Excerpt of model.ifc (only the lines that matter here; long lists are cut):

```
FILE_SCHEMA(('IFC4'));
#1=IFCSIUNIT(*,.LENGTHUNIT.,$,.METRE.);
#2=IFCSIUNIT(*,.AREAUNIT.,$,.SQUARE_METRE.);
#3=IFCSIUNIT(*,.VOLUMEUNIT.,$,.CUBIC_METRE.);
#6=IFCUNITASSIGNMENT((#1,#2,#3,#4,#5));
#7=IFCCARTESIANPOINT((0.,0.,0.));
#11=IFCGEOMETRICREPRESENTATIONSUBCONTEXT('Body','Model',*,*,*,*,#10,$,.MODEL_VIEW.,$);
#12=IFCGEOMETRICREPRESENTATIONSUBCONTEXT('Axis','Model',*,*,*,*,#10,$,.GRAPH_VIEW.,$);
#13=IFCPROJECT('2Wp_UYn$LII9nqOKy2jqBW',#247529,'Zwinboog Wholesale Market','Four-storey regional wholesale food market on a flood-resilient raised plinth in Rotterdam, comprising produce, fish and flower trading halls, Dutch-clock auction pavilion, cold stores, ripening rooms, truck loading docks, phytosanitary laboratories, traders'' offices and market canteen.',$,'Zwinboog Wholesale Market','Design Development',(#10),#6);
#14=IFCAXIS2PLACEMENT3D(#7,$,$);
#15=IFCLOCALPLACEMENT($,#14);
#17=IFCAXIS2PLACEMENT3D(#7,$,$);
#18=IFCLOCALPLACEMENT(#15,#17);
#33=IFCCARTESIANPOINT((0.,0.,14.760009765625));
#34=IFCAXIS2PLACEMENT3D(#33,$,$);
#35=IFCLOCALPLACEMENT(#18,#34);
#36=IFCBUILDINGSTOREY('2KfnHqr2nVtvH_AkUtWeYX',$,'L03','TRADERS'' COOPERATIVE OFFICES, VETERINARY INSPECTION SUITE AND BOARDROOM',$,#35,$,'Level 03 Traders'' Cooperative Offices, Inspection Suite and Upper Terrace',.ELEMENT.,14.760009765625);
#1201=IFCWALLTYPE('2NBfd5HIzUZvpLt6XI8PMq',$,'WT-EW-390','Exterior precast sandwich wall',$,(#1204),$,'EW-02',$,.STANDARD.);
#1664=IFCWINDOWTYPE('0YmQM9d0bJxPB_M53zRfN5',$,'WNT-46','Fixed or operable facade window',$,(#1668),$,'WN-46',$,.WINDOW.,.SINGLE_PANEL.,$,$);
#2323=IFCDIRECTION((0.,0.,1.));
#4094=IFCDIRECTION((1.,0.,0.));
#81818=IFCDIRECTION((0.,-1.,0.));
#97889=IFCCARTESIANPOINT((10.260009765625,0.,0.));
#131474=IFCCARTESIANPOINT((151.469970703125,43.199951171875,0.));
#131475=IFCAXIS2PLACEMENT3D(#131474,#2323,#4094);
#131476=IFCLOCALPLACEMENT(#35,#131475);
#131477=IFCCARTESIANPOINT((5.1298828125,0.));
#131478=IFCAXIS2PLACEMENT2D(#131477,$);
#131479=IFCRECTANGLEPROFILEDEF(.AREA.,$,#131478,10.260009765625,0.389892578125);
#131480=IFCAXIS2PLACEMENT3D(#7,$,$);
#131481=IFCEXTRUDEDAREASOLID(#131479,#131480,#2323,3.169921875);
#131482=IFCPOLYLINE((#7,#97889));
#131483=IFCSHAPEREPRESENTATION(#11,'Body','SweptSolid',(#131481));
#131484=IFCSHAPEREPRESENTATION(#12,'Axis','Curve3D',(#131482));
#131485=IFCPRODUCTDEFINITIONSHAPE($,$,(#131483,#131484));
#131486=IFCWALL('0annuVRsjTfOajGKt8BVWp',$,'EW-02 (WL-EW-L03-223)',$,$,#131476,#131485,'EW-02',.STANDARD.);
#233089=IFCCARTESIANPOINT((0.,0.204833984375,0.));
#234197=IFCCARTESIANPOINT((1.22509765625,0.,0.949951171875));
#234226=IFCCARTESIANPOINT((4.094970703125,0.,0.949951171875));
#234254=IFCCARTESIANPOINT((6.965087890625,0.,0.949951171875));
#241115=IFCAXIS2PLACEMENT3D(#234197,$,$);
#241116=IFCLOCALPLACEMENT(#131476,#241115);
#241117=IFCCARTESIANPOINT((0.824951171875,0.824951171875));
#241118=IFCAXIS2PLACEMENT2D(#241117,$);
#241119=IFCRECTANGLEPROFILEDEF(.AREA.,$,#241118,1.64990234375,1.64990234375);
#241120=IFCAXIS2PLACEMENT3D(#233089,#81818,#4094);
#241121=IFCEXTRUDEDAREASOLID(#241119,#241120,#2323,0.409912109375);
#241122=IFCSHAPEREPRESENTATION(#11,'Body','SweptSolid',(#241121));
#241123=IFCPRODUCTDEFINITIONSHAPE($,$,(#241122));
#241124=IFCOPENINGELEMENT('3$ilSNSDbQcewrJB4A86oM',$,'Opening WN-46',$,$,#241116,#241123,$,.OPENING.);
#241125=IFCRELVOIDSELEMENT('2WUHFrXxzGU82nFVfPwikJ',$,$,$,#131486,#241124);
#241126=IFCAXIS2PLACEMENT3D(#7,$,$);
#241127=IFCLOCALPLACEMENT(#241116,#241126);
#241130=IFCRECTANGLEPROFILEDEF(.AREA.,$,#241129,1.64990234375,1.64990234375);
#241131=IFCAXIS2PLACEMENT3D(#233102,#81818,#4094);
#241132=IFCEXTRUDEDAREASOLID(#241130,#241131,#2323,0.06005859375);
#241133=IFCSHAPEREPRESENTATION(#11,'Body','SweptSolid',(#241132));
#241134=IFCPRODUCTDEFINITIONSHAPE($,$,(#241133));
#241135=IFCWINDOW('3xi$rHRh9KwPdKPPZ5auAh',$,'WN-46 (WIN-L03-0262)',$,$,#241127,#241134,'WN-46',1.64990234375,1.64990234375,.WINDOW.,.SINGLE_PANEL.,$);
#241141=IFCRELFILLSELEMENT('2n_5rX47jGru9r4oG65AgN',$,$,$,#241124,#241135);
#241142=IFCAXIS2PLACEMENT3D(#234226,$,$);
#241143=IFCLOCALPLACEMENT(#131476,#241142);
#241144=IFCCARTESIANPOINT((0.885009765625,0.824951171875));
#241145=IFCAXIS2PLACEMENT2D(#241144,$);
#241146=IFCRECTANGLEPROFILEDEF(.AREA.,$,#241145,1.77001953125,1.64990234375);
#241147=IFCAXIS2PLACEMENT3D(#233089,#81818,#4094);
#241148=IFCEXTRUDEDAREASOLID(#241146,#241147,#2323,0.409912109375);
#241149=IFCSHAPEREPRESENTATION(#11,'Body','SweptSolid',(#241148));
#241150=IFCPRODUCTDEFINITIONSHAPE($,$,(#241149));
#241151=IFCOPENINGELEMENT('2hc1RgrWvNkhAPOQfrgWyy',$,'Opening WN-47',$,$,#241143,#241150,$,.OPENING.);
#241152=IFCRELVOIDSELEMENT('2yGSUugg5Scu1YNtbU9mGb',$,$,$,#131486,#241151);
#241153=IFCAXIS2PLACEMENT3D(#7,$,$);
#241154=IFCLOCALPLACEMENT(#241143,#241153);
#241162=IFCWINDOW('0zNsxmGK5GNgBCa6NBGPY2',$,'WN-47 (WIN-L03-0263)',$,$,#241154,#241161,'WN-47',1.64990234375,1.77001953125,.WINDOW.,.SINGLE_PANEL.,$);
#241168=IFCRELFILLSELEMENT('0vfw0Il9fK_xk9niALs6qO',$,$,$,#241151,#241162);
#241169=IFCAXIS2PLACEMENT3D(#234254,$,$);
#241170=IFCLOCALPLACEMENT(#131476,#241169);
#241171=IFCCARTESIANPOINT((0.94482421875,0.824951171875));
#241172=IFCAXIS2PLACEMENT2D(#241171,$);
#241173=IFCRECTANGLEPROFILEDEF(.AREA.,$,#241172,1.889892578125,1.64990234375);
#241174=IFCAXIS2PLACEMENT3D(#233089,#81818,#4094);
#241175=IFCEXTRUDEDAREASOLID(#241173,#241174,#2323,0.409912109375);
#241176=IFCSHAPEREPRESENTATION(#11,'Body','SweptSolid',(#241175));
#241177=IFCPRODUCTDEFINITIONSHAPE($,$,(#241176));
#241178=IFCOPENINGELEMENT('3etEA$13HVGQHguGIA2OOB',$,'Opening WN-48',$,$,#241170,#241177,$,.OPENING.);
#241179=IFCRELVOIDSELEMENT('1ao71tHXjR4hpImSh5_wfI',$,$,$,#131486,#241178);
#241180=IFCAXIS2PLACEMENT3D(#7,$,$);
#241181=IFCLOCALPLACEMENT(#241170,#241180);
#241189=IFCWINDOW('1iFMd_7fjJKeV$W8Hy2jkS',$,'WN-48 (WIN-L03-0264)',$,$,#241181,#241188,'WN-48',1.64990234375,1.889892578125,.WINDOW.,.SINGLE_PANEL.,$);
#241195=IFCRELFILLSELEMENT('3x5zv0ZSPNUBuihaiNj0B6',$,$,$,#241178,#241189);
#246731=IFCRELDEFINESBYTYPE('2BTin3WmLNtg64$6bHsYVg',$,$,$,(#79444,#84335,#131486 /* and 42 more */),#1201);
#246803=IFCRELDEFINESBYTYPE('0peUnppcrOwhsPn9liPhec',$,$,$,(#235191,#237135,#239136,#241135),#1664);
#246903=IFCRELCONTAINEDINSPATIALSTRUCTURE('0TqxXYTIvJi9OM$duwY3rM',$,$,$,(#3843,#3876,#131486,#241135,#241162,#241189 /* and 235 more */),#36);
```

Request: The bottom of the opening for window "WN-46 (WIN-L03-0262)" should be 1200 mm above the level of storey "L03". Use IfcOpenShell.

```python
import numpy as np
import ifcopenshell
import ifcopenshell.api.geometry
import ifcopenshell.geom
import ifcopenshell.util.element
import ifcopenshell.util.placement
import ifcopenshell.util.shape
import ifcopenshell.util.unit

model = ifcopenshell.open("model.ifc")
unit_scale = ifcopenshell.util.unit.calculate_unit_scale(model)

window = model.by_guid("3xi$rHRh9KwPdKPPZ5auAh")
opening = window.FillsVoids[0].RelatingOpeningElement
storey = ifcopenshell.util.element.get_container(window, ifc_class="IfcBuildingStorey")
level = ifcopenshell.util.placement.get_local_placement(storey.ObjectPlacement)[2, 3]

# The opening's origin need not be at the sill, so measure its lowest point.
shape = ifcopenshell.geom.create_shape(ifcopenshell.geom.settings(), opening)
bottom = ifcopenshell.util.shape.get_shape_bottom_elevation(shape, shape.geometry) / unit_scale
dz = level + 1.2 / unit_scale - bottom

shift = np.array([0.0, 0.0, dz])
# The window is placed relative to its opening, so it follows when the opening moves.
matrix = ifcopenshell.util.placement.get_local_placement(opening.ObjectPlacement)
matrix[:3, 3] += shift
ifcopenshell.api.geometry.edit_object_placement(
    model, product=opening, matrix=matrix, is_si=False, should_transform_children=True
)

print(f"moved by {dz * unit_scale:+.3f} m")

model.write("model_rev.ifc")
```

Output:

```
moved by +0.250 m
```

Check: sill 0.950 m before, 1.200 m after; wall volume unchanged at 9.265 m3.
